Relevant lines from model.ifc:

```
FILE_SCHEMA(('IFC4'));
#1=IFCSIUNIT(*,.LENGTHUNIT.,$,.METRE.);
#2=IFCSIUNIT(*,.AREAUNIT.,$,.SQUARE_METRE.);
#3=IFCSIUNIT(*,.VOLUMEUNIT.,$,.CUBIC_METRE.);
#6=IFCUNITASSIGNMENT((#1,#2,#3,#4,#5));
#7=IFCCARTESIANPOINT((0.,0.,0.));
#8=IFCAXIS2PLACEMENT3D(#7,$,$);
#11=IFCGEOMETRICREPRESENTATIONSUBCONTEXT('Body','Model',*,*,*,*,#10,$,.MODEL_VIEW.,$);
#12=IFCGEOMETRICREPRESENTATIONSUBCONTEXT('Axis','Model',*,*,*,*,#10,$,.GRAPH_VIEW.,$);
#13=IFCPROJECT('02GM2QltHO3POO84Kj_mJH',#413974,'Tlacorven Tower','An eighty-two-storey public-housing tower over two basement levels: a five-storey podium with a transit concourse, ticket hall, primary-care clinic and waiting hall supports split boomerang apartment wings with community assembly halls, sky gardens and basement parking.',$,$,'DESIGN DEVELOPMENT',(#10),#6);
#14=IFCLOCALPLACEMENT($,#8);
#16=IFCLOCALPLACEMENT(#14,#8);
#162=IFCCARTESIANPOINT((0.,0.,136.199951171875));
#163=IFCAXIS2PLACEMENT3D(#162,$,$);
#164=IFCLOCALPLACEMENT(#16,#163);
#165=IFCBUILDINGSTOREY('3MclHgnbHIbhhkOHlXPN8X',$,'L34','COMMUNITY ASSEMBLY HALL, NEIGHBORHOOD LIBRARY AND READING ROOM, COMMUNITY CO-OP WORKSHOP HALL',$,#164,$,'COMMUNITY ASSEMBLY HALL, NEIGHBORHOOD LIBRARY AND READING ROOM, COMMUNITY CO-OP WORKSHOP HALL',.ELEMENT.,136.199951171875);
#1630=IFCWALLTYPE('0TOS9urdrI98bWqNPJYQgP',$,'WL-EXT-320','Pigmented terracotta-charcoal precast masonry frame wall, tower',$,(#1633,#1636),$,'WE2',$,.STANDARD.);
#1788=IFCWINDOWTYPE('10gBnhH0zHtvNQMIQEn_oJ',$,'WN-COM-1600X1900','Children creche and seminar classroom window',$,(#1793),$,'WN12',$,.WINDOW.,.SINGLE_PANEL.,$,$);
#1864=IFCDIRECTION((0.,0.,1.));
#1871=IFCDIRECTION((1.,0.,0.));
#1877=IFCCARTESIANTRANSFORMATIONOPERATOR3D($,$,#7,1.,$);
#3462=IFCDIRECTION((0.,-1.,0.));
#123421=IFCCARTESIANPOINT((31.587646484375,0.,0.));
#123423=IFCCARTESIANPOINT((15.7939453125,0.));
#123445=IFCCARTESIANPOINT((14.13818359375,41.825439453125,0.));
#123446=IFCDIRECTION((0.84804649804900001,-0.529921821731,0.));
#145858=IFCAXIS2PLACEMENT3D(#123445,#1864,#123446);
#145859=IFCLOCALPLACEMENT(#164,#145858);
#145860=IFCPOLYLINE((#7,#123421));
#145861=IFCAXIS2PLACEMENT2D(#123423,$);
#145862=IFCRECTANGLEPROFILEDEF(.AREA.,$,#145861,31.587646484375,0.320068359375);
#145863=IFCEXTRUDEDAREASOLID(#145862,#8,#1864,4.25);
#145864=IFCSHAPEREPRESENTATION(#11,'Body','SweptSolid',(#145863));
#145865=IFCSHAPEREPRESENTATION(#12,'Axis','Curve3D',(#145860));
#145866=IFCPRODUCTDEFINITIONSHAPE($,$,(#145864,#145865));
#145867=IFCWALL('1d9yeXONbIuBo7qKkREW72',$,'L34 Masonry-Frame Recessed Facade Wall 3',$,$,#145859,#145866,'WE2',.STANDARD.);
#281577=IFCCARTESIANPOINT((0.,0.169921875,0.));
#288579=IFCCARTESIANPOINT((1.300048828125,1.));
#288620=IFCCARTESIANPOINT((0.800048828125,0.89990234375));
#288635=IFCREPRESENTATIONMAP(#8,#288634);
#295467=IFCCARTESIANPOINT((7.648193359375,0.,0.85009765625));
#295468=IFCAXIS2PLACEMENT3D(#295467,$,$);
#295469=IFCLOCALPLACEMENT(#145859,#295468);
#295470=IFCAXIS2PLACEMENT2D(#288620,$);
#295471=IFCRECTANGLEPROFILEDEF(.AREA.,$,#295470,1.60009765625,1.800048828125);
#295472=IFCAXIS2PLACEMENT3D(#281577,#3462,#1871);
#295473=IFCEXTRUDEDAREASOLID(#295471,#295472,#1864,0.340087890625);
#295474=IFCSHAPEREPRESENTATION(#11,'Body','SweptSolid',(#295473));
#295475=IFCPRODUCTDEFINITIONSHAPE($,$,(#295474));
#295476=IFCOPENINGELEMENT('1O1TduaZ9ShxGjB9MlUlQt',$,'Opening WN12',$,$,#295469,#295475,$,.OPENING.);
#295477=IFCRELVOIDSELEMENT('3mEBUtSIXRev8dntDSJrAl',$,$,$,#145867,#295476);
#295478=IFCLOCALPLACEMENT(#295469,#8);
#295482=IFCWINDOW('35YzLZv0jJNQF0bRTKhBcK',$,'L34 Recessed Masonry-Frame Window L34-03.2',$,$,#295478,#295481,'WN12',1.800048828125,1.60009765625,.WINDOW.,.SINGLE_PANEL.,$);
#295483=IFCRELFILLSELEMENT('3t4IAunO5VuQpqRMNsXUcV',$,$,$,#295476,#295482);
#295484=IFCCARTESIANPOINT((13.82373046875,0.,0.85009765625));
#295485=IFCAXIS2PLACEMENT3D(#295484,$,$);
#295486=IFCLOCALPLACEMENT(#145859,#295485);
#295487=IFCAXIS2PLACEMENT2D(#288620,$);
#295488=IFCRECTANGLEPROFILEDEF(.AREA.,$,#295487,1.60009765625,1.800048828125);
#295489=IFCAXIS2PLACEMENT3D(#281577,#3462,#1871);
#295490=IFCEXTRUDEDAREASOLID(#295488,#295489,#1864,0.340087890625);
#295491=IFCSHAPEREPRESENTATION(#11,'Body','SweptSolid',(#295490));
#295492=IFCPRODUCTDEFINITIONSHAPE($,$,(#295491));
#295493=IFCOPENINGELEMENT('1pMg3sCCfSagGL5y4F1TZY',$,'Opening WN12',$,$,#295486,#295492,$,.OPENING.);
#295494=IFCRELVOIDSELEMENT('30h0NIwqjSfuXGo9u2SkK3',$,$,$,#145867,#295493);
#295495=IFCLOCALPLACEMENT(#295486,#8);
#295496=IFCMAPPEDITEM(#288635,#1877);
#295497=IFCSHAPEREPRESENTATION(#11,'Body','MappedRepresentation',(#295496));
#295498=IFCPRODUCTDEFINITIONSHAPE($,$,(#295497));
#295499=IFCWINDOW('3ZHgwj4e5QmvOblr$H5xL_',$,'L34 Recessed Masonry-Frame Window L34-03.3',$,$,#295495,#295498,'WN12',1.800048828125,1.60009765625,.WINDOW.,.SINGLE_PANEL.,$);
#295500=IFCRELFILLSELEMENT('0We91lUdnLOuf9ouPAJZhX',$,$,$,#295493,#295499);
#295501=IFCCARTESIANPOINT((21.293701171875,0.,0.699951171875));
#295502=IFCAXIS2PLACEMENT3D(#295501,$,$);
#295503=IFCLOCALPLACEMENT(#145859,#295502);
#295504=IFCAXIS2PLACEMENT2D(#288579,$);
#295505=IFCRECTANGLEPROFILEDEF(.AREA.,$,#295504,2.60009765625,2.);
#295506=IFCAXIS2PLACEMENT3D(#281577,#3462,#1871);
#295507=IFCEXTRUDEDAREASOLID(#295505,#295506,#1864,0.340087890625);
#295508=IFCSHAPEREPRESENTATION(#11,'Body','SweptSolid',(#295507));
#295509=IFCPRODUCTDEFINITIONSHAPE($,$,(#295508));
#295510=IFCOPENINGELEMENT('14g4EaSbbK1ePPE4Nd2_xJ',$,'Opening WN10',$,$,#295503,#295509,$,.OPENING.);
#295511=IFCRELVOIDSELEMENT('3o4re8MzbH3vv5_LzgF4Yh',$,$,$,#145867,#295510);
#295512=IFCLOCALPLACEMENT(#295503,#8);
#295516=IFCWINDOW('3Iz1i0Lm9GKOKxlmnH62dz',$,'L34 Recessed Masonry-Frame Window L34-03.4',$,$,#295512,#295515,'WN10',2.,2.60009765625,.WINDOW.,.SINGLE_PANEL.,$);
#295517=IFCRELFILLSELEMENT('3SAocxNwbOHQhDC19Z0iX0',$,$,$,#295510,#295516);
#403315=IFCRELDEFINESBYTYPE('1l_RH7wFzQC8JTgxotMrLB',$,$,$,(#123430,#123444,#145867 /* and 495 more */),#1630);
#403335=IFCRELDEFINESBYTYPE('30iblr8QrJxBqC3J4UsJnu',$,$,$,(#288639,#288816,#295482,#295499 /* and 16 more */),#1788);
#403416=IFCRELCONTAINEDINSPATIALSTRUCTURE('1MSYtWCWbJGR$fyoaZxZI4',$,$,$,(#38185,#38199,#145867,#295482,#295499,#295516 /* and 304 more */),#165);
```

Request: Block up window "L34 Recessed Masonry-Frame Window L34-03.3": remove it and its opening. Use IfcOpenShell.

```python
import ifcopenshell
import ifcopenshell.api.feature
import ifcopenshell.api.root
import ifcopenshell.geom
import ifcopenshell.util.shape

model = ifcopenshell.open("model.ifc")
settings = ifcopenshell.geom.settings()


def volume(element):
    """Net volume in cubic metres, openings subtracted."""
    shape = ifcopenshell.geom.create_shape(settings, element)
    return ifcopenshell.util.shape.get_volume(shape.geometry)


window = model.by_guid("3ZHgwj4e5QmvOblr$H5xL_")
opening = window.FillsVoids[0].RelatingOpeningElement
wall = opening.VoidsElements[0].RelatingBuildingElement
before = volume(wall)

ifcopenshell.api.root.remove_product(model, product=window)
ifcopenshell.api.feature.remove_feature(model, feature=opening)

after = volume(wall)

print(f"wall volume {before:.3f} -> {after:.3f} m3")

model.write("model_rev.ifc")
```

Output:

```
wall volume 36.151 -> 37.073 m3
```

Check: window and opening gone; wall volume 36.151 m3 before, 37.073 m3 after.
